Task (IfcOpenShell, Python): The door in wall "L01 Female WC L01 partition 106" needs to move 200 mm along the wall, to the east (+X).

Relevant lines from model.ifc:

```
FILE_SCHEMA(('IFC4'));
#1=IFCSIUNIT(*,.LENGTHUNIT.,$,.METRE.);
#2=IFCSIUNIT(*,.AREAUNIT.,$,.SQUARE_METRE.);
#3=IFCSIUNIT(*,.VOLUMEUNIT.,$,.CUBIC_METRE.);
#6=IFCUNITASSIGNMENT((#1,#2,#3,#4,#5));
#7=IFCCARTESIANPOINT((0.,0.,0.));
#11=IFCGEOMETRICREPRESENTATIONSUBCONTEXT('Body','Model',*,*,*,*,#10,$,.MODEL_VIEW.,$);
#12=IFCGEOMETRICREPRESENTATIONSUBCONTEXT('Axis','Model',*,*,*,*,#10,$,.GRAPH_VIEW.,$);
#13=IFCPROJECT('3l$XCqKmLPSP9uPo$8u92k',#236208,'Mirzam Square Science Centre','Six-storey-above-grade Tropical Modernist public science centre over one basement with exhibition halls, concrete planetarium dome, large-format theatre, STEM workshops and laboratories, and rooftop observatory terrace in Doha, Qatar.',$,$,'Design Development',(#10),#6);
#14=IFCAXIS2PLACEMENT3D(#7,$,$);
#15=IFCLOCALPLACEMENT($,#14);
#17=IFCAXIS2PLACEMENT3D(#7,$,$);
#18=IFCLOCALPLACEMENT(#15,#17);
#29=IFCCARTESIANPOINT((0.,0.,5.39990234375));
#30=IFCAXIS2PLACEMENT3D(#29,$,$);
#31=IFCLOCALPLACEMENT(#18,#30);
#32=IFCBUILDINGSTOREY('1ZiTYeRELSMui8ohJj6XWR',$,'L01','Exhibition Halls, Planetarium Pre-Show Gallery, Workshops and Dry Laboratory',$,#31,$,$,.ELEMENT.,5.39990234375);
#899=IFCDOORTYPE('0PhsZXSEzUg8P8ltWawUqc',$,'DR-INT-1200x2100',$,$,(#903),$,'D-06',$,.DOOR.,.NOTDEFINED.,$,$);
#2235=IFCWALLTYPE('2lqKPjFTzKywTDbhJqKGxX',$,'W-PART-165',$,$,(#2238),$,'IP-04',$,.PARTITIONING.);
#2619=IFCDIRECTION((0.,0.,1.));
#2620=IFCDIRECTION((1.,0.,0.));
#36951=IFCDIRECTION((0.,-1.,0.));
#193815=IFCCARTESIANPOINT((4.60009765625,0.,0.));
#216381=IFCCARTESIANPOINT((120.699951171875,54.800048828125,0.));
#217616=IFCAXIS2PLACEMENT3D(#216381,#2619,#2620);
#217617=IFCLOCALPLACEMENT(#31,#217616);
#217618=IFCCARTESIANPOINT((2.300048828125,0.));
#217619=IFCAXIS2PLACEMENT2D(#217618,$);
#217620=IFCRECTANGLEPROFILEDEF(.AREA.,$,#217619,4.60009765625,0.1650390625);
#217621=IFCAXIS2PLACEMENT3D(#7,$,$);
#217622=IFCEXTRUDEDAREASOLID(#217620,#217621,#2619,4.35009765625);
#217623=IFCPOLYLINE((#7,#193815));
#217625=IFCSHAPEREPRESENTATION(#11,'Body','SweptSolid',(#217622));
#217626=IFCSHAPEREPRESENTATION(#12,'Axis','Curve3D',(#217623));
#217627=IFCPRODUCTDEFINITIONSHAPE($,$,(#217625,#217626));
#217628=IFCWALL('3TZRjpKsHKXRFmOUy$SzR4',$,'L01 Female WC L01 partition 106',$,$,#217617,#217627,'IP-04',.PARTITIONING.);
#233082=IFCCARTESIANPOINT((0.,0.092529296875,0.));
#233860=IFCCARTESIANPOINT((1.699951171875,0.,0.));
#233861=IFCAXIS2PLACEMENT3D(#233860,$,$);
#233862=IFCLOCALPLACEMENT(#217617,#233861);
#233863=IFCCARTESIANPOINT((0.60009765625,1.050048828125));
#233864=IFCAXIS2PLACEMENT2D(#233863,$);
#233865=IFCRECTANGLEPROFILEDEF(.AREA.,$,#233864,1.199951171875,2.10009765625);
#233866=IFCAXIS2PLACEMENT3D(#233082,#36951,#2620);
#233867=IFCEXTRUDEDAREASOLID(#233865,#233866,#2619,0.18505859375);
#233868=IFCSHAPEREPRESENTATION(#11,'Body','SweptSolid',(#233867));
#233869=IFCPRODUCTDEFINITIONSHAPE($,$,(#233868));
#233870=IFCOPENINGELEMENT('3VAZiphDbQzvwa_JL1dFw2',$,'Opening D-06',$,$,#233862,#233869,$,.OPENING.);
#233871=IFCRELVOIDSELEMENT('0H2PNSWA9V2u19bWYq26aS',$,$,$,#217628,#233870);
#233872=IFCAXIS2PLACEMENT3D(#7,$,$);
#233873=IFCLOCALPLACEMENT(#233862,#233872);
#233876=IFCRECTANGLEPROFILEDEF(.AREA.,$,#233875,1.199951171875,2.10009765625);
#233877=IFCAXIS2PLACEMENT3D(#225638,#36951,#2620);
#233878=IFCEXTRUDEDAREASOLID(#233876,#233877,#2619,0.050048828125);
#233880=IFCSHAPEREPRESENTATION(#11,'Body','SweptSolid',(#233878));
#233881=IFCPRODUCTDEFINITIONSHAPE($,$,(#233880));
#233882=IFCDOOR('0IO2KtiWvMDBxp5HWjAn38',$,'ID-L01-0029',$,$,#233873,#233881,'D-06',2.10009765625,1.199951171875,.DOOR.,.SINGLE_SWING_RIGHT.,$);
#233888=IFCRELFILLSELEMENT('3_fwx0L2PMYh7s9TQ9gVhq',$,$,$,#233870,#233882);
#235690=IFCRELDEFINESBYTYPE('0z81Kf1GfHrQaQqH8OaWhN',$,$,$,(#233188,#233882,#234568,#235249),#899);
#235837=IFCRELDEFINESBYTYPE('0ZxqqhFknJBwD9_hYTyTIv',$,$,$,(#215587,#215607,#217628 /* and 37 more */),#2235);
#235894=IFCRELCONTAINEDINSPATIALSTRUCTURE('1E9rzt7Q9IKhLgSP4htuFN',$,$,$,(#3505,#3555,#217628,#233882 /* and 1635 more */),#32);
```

```python
import ifcopenshell
import ifcopenshell.api.geometry
import ifcopenshell.util.placement

model = ifcopenshell.open("model.ifc")

door = model.by_guid("0IO2KtiWvMDBxp5HWjAn38")
opening = door.FillsVoids[0].RelatingOpeningElement
wall = opening.VoidsElements[0].RelatingBuildingElement

wall_matrix = ifcopenshell.util.placement.get_local_placement(wall.ObjectPlacement)
shift = wall_matrix[:3, 0] * 0.2
before = ifcopenshell.util.placement.get_local_placement(door.ObjectPlacement)[:3, 3].copy()

# The door is placed relative to its opening, so it follows when the opening moves.
matrix = ifcopenshell.util.placement.get_local_placement(opening.ObjectPlacement)
matrix[:3, 3] += shift
ifcopenshell.api.geometry.edit_object_placement(
    model, product=opening, matrix=matrix, is_si=False, should_transform_children=True
)

after = ifcopenshell.util.placement.get_local_placement(door.ObjectPlacement)[:3, 3]
print("door moved by", (after - before).round(3) + 0.0)

model.write("model_updated.ifc")
```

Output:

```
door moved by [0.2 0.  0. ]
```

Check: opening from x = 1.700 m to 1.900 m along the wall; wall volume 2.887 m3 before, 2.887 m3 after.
